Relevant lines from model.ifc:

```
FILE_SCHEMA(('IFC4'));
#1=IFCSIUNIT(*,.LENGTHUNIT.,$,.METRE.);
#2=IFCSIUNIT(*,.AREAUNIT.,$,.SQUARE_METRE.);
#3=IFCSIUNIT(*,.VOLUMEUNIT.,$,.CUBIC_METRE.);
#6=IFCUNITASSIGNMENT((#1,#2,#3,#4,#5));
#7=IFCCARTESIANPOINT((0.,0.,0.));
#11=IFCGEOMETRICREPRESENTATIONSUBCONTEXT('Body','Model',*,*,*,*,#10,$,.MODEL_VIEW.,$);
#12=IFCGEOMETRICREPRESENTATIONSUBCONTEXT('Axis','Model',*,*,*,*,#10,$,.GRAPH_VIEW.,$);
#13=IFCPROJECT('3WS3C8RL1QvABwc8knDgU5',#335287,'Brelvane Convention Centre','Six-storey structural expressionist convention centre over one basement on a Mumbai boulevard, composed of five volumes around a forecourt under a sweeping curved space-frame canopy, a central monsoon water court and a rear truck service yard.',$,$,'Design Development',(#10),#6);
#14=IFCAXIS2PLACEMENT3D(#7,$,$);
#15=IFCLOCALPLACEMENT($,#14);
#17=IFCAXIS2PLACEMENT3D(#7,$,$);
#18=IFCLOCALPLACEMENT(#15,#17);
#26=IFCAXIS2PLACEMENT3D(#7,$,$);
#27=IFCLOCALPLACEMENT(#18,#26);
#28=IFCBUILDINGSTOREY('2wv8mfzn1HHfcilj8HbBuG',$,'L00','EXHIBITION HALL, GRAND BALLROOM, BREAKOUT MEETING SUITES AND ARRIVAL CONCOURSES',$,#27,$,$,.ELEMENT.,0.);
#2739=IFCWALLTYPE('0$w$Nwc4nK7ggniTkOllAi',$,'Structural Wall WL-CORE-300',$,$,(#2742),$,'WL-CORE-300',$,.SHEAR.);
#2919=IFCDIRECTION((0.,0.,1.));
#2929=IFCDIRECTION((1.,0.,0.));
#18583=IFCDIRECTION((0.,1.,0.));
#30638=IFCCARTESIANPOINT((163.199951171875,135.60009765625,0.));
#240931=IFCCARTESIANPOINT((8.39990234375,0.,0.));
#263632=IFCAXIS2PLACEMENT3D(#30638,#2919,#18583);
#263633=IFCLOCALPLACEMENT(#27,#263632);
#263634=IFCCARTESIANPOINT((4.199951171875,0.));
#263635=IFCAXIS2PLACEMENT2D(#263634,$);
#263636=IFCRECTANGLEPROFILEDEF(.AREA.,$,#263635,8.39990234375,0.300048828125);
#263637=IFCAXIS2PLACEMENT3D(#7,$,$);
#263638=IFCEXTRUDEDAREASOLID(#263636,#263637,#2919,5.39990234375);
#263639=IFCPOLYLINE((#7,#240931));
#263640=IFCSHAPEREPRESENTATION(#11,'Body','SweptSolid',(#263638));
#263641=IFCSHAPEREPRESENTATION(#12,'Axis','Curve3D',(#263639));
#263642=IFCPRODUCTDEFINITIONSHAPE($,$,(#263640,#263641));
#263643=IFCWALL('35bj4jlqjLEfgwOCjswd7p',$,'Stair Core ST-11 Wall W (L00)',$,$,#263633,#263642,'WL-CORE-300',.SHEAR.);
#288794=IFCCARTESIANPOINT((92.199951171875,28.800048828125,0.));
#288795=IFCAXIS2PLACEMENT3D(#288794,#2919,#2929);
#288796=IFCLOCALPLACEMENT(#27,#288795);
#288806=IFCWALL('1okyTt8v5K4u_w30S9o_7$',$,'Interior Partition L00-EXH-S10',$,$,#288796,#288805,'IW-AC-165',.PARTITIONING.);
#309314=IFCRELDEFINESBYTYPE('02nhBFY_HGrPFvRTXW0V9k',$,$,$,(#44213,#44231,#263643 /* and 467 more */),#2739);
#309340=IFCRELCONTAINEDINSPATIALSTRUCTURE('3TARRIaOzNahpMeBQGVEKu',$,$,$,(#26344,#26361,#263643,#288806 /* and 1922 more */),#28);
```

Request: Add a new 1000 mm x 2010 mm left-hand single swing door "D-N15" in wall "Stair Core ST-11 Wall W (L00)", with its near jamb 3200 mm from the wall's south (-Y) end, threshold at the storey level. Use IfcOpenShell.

```python
import numpy as np
import ifcopenshell
import ifcopenshell.api.feature
import ifcopenshell.api.geometry
import ifcopenshell.api.root
import ifcopenshell.api.spatial
import ifcopenshell.geom
import ifcopenshell.util.element
import ifcopenshell.util.placement
import ifcopenshell.util.representation
import ifcopenshell.util.shape
import ifcopenshell.util.unit

model = ifcopenshell.open("model.ifc")
unit_scale = ifcopenshell.util.unit.calculate_unit_scale(model)
settings = ifcopenshell.geom.settings()


def volume(element):
    """Net volume in cubic metres, openings subtracted."""
    shape = ifcopenshell.geom.create_shape(settings, element)
    return ifcopenshell.util.shape.get_volume(shape.geometry)


wall = model.by_guid("35bj4jlqjLEfgwOCjswd7p")
storey = ifcopenshell.util.element.get_container(wall, ifc_class="IfcBuildingStorey")
context = ifcopenshell.util.representation.get_context(model, "Model", "Body", "MODEL_VIEW")
before = volume(wall)

width, height, from_end, sill = 1, 2.01, 3.2, 0.0  # metres

# The wall runs along its own X axis, and the end named is its -X end.
wall_shape = ifcopenshell.geom.create_shape(settings, wall)
x, y, z = ifcopenshell.util.shape.get_vertices(wall_shape.geometry).T
start = x.min() + from_end
face, thickness = float(y.min()), float(y.max() - y.min())
wall_matrix = ifcopenshell.util.placement.get_local_placement(wall.ObjectPlacement)
level = ifcopenshell.util.placement.get_local_placement(storey.ObjectPlacement)[2, 3]


def in_wall(x, y):
    """Placement at x, y metres in the wall's axes, at sill height."""
    matrix = wall_matrix.copy()
    matrix[:, 3] = wall_matrix @ np.array([x / unit_scale, y / unit_scale, 0.0, 1.0])
    matrix[2, 3] = level + sill / unit_scale
    return matrix


# Opening: a box that overshoots both wall faces by 50 mm.
opening = ifcopenshell.api.root.create_entity(model, ifc_class="IfcOpeningElement", predefined_type="OPENING")
box = ifcopenshell.api.geometry.add_wall_representation(
    model, context=context, length=width, height=height, thickness=thickness + 0.1
)
ifcopenshell.api.geometry.assign_representation(model, product=opening, representation=box)
ifcopenshell.api.geometry.edit_object_placement(model, product=opening, matrix=in_wall(start, face - 0.05), is_si=False)
ifcopenshell.api.feature.add_feature(model, feature=opening, element=wall)

door = ifcopenshell.api.root.create_entity(model, ifc_class="IfcDoor", name="D-N15", predefined_type="DOOR")
door.OverallWidth, door.OverallHeight = width / unit_scale, height / unit_scale
door.OperationType = "SINGLE_SWING_LEFT"
body = ifcopenshell.api.geometry.add_door_representation(
    model,
    context=context,
    overall_width=door.OverallWidth,
    overall_height=door.OverallHeight,
    operation_type="SINGLE_SWING_LEFT",
    lining_properties={"LiningDepth": thickness / unit_scale, "ThresholdDepth": thickness / unit_scale},
)
ifcopenshell.api.geometry.assign_representation(model, product=door, representation=body)
ifcopenshell.api.spatial.assign_container(model, products=[door], relating_structure=storey)
ifcopenshell.api.feature.add_filling(model, opening=opening, element=door)

# The lining spans the wall, so the door starts at the wall face.
ifcopenshell.api.geometry.edit_object_placement(model, product=door, matrix=in_wall(start, face), is_si=False)

after = volume(wall)

print(f"wall volume {before:.3f} -> {after:.3f} m3")

model.write("model-out.ifc")
```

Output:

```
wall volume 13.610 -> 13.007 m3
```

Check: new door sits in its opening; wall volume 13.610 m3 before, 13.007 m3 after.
